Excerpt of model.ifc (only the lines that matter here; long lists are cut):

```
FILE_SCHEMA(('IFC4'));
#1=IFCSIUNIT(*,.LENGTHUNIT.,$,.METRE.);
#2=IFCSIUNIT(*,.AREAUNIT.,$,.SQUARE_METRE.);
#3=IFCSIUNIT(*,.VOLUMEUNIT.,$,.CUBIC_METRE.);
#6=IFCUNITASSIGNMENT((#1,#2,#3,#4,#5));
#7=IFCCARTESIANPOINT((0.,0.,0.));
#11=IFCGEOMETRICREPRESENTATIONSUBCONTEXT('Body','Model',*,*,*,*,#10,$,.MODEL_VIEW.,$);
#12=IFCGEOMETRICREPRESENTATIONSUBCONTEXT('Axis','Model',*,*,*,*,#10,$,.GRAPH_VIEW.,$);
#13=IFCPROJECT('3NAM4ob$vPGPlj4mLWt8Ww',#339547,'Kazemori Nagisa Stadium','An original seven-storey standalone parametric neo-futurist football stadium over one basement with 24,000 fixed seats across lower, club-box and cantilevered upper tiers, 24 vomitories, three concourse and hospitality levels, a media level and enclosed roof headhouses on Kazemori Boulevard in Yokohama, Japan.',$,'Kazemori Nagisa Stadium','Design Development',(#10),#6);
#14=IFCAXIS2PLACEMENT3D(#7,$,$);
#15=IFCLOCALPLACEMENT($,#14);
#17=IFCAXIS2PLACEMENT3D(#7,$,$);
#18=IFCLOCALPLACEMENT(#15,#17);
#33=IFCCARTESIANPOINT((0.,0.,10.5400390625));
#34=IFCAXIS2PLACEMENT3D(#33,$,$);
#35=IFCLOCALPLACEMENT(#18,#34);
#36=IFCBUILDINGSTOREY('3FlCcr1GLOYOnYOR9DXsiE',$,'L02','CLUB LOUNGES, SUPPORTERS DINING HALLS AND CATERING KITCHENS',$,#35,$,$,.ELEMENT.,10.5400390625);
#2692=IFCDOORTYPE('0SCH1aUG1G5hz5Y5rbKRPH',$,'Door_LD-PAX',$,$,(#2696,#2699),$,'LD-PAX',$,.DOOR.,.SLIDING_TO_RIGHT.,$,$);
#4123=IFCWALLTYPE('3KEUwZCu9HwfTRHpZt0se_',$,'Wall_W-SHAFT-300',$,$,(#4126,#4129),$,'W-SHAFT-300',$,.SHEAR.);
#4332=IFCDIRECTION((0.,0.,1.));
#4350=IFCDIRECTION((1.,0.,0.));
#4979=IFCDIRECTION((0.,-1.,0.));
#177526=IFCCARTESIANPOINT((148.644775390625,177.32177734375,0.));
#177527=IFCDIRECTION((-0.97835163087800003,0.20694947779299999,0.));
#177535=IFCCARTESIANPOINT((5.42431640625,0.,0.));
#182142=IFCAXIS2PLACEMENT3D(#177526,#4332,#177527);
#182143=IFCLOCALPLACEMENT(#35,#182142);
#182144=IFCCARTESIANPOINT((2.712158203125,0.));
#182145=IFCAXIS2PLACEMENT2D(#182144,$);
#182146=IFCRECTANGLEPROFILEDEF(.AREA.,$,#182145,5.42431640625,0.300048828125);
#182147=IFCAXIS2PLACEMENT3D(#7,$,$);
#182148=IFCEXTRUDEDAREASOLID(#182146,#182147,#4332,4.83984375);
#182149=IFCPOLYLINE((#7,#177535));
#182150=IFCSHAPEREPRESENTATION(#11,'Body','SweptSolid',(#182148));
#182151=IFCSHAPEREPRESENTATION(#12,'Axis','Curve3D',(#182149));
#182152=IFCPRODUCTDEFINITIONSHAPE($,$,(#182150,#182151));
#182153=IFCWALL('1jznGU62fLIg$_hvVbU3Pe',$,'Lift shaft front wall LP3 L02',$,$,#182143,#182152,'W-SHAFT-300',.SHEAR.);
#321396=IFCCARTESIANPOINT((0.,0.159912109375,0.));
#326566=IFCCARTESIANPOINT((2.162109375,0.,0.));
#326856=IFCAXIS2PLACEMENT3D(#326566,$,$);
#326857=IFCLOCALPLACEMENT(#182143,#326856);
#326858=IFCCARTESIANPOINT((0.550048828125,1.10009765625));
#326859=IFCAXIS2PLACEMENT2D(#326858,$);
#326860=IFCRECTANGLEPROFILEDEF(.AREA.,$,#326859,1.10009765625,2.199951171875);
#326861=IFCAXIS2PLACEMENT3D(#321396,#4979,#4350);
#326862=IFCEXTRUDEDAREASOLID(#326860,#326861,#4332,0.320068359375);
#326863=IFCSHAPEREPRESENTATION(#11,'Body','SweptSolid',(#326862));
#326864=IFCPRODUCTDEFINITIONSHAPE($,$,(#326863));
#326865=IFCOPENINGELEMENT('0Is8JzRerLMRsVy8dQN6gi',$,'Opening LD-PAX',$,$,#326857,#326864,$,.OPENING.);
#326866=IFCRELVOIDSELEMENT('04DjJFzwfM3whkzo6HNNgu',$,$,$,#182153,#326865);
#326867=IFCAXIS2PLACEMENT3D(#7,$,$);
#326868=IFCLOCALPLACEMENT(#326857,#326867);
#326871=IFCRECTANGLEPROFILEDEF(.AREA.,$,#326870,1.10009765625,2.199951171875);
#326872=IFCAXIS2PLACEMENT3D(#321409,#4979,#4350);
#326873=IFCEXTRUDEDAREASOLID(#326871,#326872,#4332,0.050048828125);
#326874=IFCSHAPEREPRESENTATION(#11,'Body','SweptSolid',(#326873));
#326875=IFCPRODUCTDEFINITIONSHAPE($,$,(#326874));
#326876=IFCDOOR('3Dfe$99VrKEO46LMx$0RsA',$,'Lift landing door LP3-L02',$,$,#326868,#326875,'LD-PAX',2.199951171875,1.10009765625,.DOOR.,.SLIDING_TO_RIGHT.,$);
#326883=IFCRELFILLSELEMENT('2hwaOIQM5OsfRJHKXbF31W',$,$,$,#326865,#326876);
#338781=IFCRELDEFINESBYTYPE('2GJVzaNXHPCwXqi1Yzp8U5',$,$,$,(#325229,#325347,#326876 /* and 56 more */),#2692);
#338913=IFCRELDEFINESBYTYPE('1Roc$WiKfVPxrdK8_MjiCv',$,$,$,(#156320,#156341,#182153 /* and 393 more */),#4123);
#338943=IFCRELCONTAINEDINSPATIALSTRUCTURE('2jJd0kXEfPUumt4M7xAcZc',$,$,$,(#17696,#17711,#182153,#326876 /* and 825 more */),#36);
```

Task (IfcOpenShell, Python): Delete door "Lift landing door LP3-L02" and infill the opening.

```python
import ifcopenshell
import ifcopenshell.api.feature
import ifcopenshell.api.root
import ifcopenshell.geom
import ifcopenshell.util.shape

model = ifcopenshell.open("model.ifc")
settings = ifcopenshell.geom.settings()


def volume(element):
    """Net volume in cubic metres, openings subtracted."""
    shape = ifcopenshell.geom.create_shape(settings, element)
    return ifcopenshell.util.shape.get_volume(shape.geometry)


door = model.by_id(326876)
opening = door.FillsVoids[0].RelatingOpeningElement
wall = opening.VoidsElements[0].RelatingBuildingElement
before = volume(wall)

ifcopenshell.api.root.remove_product(model, product=door)
ifcopenshell.api.feature.remove_feature(model, feature=opening)

after = volume(wall)

print(f"wall volume {before:.3f} -> {after:.3f} m3")

model.write("model_rev.ifc")
```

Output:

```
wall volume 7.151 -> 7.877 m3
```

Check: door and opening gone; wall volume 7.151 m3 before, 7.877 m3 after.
